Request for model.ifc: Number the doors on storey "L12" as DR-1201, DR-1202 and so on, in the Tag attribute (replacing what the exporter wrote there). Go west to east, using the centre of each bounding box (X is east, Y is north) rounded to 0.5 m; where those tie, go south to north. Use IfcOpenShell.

First a look at what the model holds.

```python
import ifcopenshell
import ifcopenshell.util.element
import ifcopenshell.util.placement

model = ifcopenshell.open("model.ifc")
print(model.schema)
storey = next(s for s in model.by_type("IfcBuildingStorey") if s.Name == "L12")
doors = [e for e in ifcopenshell.util.element.get_decomposition(storey) if e.is_a("IfcDoor")]
for e in sorted(doors, key=lambda e: e.id()):
    origin = ifcopenshell.util.placement.get_local_placement(e.ObjectPlacement)[:3, 3]
    print(e.id(), e.Tag, e.Name, origin.round(2) + 0.0, sep=" | ")
```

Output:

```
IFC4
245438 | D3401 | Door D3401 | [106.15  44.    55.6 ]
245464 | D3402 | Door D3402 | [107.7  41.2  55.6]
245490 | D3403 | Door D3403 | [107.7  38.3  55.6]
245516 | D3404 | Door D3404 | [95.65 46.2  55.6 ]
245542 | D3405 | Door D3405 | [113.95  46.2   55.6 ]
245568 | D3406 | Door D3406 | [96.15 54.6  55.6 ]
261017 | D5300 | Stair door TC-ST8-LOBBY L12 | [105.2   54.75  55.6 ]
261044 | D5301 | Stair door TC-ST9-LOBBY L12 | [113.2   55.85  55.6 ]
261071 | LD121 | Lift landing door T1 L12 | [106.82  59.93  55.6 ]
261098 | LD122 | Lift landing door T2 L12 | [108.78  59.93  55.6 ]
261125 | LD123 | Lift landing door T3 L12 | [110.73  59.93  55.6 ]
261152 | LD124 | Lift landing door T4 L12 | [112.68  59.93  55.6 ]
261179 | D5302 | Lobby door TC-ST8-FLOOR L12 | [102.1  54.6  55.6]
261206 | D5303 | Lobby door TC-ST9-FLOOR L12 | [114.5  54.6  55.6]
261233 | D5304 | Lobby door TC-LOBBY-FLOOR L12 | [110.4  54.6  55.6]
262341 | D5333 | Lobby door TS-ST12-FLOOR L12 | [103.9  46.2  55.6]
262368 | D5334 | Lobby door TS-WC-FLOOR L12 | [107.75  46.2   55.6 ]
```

```python
import ifcopenshell
import ifcopenshell.geom
import ifcopenshell.util.element
import ifcopenshell.util.shape

model = ifcopenshell.open("model.ifc")
settings = ifcopenshell.geom.settings()
settings.set("use-world-coords", True)


def centre(element):
    shape = ifcopenshell.geom.create_shape(settings, element)
    return ifcopenshell.util.shape.get_bbox_centroid(shape.geometry)


storey = next(s for s in model.by_type("IfcBuildingStorey") if s.Name == "L12")
doors = [e for e in ifcopenshell.util.element.get_decomposition(storey) if e.is_a("IfcDoor")]

# Insertion points can sit at a corner or the storey origin, so sort by the geometry (in metres).
centres = {e: centre(e) for e in doors}
doors.sort(key=lambda e: (round(centres[e][0] / 0.5), centres[e][1]))

for i, e in enumerate(doors, start=1):
    number = f"DR-12{i:02d}"
    e.Tag = number
    print(e.id(), number)

model.write("model_v2.ifc")
```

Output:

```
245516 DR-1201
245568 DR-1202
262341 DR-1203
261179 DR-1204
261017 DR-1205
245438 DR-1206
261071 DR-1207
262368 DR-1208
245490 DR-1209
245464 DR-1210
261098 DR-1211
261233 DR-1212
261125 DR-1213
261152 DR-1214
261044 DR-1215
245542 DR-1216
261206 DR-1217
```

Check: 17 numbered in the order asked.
